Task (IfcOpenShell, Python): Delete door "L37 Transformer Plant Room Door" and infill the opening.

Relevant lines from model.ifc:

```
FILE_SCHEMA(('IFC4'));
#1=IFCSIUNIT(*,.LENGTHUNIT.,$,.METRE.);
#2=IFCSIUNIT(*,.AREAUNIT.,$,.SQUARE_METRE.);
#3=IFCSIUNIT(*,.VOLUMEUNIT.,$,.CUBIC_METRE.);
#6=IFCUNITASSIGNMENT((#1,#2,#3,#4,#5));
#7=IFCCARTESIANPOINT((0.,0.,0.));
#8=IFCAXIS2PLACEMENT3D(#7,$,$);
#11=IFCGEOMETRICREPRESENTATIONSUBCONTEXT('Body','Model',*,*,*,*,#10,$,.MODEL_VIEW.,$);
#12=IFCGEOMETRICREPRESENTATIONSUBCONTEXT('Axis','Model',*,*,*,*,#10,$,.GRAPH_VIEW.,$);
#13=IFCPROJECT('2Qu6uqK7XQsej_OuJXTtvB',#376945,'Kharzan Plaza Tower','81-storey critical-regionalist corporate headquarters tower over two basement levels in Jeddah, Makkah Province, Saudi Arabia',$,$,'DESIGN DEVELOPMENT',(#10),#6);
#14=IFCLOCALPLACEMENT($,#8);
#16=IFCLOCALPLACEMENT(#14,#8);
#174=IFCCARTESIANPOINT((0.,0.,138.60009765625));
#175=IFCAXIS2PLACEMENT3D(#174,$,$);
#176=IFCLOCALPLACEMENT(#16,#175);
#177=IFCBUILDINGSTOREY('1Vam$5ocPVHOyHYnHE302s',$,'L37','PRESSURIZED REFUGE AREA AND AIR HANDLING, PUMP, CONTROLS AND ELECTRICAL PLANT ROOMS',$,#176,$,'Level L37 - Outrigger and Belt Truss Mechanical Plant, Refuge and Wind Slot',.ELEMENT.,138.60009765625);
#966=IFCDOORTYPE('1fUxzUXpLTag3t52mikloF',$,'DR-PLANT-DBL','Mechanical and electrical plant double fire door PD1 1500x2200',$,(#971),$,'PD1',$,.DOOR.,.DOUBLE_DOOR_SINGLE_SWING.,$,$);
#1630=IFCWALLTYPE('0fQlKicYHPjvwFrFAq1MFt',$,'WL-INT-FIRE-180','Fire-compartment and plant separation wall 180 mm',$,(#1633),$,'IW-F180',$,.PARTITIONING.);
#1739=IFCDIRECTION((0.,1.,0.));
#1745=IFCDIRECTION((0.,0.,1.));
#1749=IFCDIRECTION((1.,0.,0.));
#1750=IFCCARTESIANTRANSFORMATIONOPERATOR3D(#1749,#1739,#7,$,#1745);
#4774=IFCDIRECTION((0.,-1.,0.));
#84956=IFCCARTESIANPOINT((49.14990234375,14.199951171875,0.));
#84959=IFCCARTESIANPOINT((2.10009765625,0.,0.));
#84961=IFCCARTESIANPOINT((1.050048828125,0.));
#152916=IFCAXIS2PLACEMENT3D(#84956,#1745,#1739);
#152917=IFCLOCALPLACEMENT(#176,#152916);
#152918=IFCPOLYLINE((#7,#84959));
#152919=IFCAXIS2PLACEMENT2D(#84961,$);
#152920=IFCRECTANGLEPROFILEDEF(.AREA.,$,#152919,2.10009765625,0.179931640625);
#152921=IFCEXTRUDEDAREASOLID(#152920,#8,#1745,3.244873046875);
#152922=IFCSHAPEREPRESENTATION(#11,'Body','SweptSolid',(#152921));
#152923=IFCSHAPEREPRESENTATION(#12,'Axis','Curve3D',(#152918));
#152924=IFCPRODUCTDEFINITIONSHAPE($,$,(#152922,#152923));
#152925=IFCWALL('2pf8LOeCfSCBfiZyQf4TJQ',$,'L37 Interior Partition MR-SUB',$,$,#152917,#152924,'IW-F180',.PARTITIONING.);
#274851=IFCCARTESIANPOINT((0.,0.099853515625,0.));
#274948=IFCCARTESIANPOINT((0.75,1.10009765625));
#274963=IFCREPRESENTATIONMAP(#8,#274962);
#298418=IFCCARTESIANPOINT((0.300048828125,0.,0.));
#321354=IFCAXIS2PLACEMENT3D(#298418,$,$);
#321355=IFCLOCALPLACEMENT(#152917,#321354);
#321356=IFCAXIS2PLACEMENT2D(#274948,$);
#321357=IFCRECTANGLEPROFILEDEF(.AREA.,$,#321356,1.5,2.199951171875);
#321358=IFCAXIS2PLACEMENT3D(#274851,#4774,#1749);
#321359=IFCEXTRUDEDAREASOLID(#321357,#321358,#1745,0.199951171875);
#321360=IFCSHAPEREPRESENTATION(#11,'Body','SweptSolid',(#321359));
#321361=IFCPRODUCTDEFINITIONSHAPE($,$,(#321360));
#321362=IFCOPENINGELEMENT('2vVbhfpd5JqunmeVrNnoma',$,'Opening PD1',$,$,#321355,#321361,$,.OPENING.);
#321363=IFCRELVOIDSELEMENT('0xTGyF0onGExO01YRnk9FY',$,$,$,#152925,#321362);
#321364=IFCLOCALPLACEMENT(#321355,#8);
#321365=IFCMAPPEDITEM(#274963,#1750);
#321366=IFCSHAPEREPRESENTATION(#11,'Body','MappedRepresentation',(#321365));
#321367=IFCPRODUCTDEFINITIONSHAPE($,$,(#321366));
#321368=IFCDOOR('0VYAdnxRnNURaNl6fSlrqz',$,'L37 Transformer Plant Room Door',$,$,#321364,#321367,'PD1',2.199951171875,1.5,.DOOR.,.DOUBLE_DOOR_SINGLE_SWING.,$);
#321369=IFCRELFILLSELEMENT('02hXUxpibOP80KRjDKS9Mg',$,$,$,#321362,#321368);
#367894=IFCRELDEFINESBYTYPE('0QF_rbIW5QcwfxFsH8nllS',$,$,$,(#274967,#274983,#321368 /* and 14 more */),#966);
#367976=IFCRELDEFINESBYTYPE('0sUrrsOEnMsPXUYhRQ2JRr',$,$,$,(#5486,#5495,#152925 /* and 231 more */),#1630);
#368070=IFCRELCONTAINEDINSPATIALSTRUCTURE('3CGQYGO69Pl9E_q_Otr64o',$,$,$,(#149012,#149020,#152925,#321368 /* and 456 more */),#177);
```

```python
import ifcopenshell
import ifcopenshell.api.feature
import ifcopenshell.api.root
import ifcopenshell.geom
import ifcopenshell.util.shape

model = ifcopenshell.open("model.ifc")
settings = ifcopenshell.geom.settings()


def volume(element):
    """Net volume in cubic metres, openings subtracted."""
    shape = ifcopenshell.geom.create_shape(settings, element)
    return ifcopenshell.util.shape.get_volume(shape.geometry)


door = model.by_id(321368)
opening = door.FillsVoids[0].RelatingOpeningElement
wall = opening.VoidsElements[0].RelatingBuildingElement
before = volume(wall)

ifcopenshell.api.root.remove_product(model, product=door)
ifcopenshell.api.feature.remove_feature(model, feature=opening)

after = volume(wall)

print(f"wall volume {before:.3f} -> {after:.3f} m3")

model.write("model_v2.ifc")
```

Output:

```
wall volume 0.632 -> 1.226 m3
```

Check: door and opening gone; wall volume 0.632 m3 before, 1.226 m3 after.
